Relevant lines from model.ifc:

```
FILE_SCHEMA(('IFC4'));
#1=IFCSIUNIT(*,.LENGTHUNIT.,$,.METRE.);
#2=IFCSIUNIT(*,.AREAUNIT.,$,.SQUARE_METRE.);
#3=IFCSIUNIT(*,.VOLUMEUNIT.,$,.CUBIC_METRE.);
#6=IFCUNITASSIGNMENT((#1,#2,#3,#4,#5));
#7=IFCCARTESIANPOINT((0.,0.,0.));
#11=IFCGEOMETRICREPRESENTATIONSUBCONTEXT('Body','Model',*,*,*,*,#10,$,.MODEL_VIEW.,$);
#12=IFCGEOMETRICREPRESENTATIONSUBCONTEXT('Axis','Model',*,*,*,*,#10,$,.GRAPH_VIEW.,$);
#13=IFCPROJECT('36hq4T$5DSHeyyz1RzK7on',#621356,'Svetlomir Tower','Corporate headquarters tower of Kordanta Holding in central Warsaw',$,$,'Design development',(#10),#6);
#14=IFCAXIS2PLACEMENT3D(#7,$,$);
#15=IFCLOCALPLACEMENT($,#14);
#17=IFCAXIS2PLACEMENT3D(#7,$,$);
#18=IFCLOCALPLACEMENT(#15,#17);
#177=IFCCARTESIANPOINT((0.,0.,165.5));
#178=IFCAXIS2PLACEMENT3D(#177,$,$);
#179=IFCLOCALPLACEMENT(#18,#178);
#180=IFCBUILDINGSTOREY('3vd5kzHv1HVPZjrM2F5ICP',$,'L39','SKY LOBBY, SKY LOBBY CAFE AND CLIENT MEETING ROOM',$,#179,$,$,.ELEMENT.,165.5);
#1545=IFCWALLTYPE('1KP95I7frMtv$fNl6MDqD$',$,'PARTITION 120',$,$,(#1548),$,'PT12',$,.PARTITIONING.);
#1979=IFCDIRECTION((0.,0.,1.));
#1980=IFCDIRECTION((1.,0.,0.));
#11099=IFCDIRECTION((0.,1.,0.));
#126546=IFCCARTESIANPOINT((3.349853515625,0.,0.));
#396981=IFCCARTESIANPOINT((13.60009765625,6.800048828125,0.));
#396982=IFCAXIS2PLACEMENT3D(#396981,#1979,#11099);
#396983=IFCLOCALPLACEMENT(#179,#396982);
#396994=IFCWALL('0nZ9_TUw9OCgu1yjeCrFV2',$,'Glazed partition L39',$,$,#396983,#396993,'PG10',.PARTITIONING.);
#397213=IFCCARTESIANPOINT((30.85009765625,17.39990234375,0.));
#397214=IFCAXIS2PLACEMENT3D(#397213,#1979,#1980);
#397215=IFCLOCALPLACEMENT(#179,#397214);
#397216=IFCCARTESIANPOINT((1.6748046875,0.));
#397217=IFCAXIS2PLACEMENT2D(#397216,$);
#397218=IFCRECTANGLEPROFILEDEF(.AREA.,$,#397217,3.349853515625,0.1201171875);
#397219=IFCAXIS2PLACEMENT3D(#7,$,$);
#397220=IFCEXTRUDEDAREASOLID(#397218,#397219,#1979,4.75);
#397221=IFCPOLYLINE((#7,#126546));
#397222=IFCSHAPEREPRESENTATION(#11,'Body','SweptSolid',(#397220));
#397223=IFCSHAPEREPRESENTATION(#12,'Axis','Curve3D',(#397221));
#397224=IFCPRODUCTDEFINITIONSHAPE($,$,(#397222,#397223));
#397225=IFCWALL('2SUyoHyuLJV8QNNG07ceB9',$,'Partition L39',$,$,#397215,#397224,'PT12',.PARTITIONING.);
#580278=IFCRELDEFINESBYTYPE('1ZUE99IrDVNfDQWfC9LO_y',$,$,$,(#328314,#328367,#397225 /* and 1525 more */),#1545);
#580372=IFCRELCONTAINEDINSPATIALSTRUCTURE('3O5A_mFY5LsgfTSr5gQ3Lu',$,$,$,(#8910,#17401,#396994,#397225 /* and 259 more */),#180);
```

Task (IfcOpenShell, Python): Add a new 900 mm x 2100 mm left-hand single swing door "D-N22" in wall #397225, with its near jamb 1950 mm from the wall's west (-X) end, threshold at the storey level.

```python
import numpy as np
import ifcopenshell
import ifcopenshell.api.feature
import ifcopenshell.api.geometry
import ifcopenshell.api.root
import ifcopenshell.api.spatial
import ifcopenshell.geom
import ifcopenshell.util.element
import ifcopenshell.util.placement
import ifcopenshell.util.representation
import ifcopenshell.util.shape
import ifcopenshell.util.unit

model = ifcopenshell.open("model.ifc")
unit_scale = ifcopenshell.util.unit.calculate_unit_scale(model)
settings = ifcopenshell.geom.settings()


def volume(element):
    """Net volume in cubic metres, openings subtracted."""
    shape = ifcopenshell.geom.create_shape(settings, element)
    return ifcopenshell.util.shape.get_volume(shape.geometry)


wall = model.by_id(397225)
storey = ifcopenshell.util.element.get_container(wall, ifc_class="IfcBuildingStorey")
context = ifcopenshell.util.representation.get_context(model, "Model", "Body", "MODEL_VIEW")
before = volume(wall)

width, height, from_end, sill = 0.9, 2.1, 1.95, 0.0  # metres

# The wall runs along its own X axis, and the end named is its -X end.
wall_shape = ifcopenshell.geom.create_shape(settings, wall)
x, y, z = ifcopenshell.util.shape.get_vertices(wall_shape.geometry).T
start = x.min() + from_end
face, thickness = float(y.min()), float(y.max() - y.min())
wall_matrix = ifcopenshell.util.placement.get_local_placement(wall.ObjectPlacement)
level = ifcopenshell.util.placement.get_local_placement(storey.ObjectPlacement)[2, 3]


def in_wall(x, y):
    """Placement at x, y metres in the wall's axes, at sill height."""
    matrix = wall_matrix.copy()
    matrix[:, 3] = wall_matrix @ np.array([x / unit_scale, y / unit_scale, 0.0, 1.0])
    matrix[2, 3] = level + sill / unit_scale
    return matrix


# Opening: a box that overshoots both wall faces by 50 mm.
opening = ifcopenshell.api.root.create_entity(model, ifc_class="IfcOpeningElement", predefined_type="OPENING")
box = ifcopenshell.api.geometry.add_wall_representation(
    model, context=context, length=width, height=height, thickness=thickness + 0.1
)
ifcopenshell.api.geometry.assign_representation(model, product=opening, representation=box)
ifcopenshell.api.geometry.edit_object_placement(model, product=opening, matrix=in_wall(start, face - 0.05), is_si=False)
ifcopenshell.api.feature.add_feature(model, feature=opening, element=wall)

door = ifcopenshell.api.root.create_entity(model, ifc_class="IfcDoor", name="D-N22", predefined_type="DOOR")
door.OverallWidth, door.OverallHeight = width / unit_scale, height / unit_scale
door.OperationType = "SINGLE_SWING_LEFT"
body = ifcopenshell.api.geometry.add_door_representation(
    model,
    context=context,
    overall_width=door.OverallWidth,
    overall_height=door.OverallHeight,
    operation_type="SINGLE_SWING_LEFT",
    lining_properties={"LiningDepth": thickness / unit_scale, "ThresholdDepth": thickness / unit_scale},
)
ifcopenshell.api.geometry.assign_representation(model, product=door, representation=body)
ifcopenshell.api.spatial.assign_container(model, products=[door], relating_structure=storey)
ifcopenshell.api.feature.add_filling(model, opening=opening, element=door)

# The lining spans the wall, so the door starts at the wall face.
ifcopenshell.api.geometry.edit_object_placement(model, product=door, matrix=in_wall(start, face), is_si=False)

after = volume(wall)

print(f"wall volume {before:.3f} -> {after:.3f} m3")

model.write("model_edited.ifc")
```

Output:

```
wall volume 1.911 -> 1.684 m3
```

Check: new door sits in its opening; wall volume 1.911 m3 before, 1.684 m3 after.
